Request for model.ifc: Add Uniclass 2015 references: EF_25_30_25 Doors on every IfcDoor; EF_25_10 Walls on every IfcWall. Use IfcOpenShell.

First a look at what the model holds.

```python
import ifcopenshell

model = ifcopenshell.open("model.ifc")
print(model.schema)
print("classifications:", [c.Name for c in model.by_type("IfcClassification")])
for ifc_class in ("IfcDoor", "IfcRoof", "IfcStair", "IfcWall", "IfcWindow"):
    print(ifc_class, len(model.by_type(ifc_class)))
```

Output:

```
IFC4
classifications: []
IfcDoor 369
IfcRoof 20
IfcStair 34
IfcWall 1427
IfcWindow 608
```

```python
import ifcopenshell
import ifcopenshell.api.classification

model = ifcopenshell.open("model.ifc")

system = ifcopenshell.api.classification.add_classification(model, classification="Uniclass 2015")

codes = {
    "IfcDoor": ("EF_25_30_25", "Doors"),
    "IfcWall": ("EF_25_10", "Walls"),
}
for ifc_class, (code, name) in codes.items():
    products = model.by_type(ifc_class)
    ifcopenshell.api.classification.add_reference(
        model, products=products, classification=system, identification=code, name=name
    )
    print(code, len(products))

model.write("model_edited.ifc")
```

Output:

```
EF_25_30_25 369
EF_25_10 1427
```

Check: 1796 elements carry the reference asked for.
